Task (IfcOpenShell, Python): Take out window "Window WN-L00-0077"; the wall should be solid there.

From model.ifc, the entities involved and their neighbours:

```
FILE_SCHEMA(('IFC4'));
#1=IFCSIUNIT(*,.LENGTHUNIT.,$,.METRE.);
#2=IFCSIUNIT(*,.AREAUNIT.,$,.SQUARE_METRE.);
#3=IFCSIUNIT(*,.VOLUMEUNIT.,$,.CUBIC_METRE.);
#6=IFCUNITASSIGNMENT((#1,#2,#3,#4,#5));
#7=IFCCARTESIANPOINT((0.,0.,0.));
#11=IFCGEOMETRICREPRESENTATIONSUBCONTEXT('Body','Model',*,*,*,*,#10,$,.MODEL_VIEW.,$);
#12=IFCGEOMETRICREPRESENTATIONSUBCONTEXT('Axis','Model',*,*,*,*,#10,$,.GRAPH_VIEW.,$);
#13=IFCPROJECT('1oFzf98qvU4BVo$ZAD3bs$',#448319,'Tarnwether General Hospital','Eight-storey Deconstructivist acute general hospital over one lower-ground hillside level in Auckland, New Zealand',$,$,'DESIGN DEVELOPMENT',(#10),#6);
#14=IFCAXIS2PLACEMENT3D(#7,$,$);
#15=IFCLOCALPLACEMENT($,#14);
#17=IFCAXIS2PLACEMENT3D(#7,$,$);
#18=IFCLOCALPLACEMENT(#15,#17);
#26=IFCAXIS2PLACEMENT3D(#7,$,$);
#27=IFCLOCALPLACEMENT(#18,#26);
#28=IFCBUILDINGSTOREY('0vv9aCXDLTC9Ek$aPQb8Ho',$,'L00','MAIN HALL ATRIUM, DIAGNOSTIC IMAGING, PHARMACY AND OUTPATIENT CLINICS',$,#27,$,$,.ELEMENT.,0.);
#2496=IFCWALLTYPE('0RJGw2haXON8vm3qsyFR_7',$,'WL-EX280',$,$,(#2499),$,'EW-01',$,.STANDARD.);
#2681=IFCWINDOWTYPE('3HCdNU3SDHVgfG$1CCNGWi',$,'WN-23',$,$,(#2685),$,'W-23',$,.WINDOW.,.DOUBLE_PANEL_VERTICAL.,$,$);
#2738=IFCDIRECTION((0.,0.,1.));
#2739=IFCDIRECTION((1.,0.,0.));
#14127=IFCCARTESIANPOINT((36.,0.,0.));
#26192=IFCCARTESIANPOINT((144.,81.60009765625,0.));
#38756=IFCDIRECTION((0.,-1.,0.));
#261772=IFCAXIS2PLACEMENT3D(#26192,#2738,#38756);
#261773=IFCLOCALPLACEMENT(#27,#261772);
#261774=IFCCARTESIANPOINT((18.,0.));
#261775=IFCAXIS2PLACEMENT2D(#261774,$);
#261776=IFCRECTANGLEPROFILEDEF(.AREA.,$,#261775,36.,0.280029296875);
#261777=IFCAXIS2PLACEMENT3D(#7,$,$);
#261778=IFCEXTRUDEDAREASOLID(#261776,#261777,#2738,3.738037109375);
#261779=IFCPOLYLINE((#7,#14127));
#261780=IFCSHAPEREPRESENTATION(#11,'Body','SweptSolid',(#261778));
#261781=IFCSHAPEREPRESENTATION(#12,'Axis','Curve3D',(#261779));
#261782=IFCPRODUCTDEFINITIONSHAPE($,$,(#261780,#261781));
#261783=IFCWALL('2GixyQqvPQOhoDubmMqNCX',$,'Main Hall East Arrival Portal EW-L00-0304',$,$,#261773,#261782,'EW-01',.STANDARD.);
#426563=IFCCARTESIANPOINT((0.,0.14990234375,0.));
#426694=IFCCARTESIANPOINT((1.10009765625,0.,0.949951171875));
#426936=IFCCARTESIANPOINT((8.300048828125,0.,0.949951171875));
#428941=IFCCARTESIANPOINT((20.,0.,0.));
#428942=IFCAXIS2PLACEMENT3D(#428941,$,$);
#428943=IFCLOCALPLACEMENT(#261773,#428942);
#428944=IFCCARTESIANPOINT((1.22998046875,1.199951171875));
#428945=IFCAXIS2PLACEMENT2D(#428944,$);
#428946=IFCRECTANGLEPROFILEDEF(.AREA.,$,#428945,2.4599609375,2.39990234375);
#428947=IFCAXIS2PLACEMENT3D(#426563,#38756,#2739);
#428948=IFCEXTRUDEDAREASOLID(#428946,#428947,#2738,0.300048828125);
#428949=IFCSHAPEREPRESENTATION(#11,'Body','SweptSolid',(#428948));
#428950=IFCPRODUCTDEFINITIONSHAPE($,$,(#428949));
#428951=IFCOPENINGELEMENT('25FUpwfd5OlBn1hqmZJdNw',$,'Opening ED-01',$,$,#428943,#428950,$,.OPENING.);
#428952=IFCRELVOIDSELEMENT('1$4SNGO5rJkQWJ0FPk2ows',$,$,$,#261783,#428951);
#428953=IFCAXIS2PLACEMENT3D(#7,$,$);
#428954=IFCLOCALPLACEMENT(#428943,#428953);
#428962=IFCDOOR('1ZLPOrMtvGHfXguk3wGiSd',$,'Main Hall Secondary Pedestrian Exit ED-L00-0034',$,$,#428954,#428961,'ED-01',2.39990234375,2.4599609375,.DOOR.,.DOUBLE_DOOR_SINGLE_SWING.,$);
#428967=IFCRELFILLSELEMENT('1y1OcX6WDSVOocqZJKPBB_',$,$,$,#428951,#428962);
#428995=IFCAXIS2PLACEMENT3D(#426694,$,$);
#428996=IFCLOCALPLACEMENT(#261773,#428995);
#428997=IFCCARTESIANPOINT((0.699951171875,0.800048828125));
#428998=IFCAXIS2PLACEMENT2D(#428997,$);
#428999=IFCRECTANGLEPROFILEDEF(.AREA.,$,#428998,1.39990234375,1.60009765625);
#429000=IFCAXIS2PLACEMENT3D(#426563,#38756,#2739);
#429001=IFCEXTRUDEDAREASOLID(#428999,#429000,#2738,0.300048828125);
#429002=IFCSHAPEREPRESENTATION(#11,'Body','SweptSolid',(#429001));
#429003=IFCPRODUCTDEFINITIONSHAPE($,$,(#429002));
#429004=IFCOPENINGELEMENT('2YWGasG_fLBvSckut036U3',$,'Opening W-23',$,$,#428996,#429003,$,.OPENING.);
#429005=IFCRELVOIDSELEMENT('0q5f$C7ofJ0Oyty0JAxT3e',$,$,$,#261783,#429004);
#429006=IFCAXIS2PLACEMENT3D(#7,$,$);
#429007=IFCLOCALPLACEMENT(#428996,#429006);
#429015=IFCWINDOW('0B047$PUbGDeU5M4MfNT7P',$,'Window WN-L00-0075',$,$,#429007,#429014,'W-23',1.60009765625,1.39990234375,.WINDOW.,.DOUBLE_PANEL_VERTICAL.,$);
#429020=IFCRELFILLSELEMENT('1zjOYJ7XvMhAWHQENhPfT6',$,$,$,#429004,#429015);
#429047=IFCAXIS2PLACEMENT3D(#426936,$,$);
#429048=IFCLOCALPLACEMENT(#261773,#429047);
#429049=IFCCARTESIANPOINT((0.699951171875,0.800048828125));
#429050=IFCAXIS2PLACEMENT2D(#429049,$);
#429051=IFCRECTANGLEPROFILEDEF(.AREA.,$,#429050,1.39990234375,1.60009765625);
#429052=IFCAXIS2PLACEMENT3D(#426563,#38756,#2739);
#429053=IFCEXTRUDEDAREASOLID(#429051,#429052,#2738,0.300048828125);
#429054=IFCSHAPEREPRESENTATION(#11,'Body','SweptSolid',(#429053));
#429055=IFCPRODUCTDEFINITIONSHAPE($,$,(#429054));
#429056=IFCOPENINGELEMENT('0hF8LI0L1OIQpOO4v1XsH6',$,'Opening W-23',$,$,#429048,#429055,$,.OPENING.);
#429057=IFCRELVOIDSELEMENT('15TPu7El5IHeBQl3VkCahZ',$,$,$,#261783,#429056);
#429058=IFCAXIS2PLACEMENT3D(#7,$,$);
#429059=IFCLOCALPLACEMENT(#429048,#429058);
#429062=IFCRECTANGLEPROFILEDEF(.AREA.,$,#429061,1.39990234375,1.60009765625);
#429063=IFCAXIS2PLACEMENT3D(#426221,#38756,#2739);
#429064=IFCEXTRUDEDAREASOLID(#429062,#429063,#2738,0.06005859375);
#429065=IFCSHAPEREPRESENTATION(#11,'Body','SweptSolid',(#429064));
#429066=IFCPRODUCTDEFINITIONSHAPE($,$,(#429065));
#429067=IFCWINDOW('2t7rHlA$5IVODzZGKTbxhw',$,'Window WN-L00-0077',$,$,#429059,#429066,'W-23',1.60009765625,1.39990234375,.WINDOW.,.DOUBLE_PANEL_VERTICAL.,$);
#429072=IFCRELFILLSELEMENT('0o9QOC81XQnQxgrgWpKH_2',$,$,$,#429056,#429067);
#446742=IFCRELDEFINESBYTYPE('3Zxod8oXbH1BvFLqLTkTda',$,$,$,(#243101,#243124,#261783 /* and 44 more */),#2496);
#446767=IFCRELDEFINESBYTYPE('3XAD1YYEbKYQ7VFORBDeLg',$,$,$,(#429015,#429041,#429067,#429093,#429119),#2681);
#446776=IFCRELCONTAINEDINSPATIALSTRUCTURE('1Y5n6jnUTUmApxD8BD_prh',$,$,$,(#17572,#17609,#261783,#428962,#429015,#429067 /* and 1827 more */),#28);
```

```python
import ifcopenshell
import ifcopenshell.api.feature
import ifcopenshell.api.root
import ifcopenshell.geom
import ifcopenshell.util.shape

model = ifcopenshell.open("model.ifc")
settings = ifcopenshell.geom.settings()


def volume(element):
    """Net volume in cubic metres, openings subtracted."""
    shape = ifcopenshell.geom.create_shape(settings, element)
    return ifcopenshell.util.shape.get_volume(shape.geometry)


window = model.by_id(429067)
opening = window.FillsVoids[0].RelatingOpeningElement
wall = opening.VoidsElements[0].RelatingBuildingElement
before = volume(wall)

ifcopenshell.api.root.remove_product(model, product=window)
ifcopenshell.api.feature.remove_feature(model, feature=opening)

after = volume(wall)

print(f"wall volume {before:.3f} -> {after:.3f} m3")

model.write("model_rev.ifc")
```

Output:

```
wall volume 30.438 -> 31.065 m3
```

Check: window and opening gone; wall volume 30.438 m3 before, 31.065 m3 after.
